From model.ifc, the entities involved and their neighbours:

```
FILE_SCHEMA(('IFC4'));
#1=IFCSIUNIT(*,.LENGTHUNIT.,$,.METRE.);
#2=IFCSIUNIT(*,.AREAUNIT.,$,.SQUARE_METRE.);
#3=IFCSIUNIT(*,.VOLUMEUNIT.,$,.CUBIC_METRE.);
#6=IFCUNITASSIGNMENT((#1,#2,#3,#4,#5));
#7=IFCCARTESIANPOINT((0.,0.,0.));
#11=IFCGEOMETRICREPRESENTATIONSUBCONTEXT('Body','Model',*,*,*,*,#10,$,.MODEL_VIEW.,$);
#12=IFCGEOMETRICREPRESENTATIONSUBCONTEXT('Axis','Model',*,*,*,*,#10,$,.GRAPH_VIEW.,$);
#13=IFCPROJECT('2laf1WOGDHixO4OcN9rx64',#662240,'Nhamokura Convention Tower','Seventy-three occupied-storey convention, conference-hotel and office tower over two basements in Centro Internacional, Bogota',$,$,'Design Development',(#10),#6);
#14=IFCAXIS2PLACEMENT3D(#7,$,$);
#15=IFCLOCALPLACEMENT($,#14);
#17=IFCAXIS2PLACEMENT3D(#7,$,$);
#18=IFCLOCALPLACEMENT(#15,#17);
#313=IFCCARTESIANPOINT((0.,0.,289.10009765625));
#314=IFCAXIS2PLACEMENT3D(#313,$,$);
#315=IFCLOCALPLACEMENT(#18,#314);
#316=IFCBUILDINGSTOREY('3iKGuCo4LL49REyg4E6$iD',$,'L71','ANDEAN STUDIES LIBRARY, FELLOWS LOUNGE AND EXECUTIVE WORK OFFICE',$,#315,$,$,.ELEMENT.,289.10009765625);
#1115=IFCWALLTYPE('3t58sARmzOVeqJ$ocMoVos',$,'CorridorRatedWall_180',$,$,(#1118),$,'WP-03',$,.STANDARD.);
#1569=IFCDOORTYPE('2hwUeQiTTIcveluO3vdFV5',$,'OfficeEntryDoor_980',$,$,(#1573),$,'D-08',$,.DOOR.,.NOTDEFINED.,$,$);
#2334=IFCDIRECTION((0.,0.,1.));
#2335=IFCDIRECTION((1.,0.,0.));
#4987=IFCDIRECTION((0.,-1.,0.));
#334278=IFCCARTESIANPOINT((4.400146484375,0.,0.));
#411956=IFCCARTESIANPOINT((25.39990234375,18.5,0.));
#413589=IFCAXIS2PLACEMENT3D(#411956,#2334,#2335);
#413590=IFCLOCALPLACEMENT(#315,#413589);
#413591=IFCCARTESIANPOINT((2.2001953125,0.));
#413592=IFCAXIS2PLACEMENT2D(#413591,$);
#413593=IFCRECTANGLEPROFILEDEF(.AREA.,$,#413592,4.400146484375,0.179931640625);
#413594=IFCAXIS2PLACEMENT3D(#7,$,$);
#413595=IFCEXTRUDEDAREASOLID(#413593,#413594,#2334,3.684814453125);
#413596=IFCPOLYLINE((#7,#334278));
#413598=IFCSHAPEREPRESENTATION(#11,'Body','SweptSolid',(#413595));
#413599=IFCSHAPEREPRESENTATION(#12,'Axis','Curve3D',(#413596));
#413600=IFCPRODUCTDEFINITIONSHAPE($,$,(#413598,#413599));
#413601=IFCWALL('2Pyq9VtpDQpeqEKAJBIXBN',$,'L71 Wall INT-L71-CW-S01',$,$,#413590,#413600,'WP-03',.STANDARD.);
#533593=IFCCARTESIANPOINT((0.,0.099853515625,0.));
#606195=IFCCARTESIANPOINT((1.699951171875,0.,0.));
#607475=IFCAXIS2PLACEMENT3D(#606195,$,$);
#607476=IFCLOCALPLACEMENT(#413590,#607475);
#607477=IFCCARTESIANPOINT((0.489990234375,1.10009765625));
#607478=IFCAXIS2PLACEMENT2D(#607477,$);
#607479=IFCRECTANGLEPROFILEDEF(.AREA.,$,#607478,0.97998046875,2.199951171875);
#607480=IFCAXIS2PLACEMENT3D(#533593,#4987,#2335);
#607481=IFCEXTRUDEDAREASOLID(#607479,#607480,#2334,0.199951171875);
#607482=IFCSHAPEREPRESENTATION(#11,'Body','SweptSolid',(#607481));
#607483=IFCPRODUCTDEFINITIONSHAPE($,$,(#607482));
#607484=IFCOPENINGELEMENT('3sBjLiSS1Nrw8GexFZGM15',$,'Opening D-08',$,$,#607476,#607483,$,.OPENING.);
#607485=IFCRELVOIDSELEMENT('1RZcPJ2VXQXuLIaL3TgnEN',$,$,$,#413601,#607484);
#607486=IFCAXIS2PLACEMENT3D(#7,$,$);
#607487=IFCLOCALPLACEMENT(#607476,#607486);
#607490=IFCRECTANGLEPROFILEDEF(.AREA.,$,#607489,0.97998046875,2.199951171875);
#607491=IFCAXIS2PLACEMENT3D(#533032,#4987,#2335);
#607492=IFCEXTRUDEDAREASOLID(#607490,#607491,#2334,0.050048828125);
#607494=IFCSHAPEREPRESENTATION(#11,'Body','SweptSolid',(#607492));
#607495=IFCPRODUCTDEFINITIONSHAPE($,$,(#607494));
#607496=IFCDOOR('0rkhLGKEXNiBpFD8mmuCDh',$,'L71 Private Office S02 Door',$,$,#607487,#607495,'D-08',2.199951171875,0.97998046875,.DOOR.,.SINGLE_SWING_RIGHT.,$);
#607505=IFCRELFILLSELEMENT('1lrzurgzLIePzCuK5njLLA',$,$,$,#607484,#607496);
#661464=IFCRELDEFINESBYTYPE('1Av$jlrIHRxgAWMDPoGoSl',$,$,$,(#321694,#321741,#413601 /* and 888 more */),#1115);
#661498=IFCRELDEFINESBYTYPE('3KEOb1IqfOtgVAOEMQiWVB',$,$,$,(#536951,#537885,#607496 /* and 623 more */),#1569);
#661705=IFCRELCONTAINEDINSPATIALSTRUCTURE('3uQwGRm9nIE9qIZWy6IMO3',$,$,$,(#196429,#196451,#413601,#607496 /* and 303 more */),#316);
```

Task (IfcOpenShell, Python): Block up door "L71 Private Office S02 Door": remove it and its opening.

```python
import ifcopenshell
import ifcopenshell.api.feature
import ifcopenshell.api.root
import ifcopenshell.geom
import ifcopenshell.util.shape

model = ifcopenshell.open("model.ifc")
settings = ifcopenshell.geom.settings()


def volume(element):
    """Net volume in cubic metres, openings subtracted."""
    shape = ifcopenshell.geom.create_shape(settings, element)
    return ifcopenshell.util.shape.get_volume(shape.geometry)


door = model.by_id(607496)
opening = door.FillsVoids[0].RelatingOpeningElement
wall = opening.VoidsElements[0].RelatingBuildingElement
before = volume(wall)

ifcopenshell.api.root.remove_product(model, product=door)
ifcopenshell.api.feature.remove_feature(model, feature=opening)

after = volume(wall)

print(f"wall volume {before:.3f} -> {after:.3f} m3")

model.write("model_edited.ifc")
```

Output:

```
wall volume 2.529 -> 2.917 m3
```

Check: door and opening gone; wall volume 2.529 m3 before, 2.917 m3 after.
